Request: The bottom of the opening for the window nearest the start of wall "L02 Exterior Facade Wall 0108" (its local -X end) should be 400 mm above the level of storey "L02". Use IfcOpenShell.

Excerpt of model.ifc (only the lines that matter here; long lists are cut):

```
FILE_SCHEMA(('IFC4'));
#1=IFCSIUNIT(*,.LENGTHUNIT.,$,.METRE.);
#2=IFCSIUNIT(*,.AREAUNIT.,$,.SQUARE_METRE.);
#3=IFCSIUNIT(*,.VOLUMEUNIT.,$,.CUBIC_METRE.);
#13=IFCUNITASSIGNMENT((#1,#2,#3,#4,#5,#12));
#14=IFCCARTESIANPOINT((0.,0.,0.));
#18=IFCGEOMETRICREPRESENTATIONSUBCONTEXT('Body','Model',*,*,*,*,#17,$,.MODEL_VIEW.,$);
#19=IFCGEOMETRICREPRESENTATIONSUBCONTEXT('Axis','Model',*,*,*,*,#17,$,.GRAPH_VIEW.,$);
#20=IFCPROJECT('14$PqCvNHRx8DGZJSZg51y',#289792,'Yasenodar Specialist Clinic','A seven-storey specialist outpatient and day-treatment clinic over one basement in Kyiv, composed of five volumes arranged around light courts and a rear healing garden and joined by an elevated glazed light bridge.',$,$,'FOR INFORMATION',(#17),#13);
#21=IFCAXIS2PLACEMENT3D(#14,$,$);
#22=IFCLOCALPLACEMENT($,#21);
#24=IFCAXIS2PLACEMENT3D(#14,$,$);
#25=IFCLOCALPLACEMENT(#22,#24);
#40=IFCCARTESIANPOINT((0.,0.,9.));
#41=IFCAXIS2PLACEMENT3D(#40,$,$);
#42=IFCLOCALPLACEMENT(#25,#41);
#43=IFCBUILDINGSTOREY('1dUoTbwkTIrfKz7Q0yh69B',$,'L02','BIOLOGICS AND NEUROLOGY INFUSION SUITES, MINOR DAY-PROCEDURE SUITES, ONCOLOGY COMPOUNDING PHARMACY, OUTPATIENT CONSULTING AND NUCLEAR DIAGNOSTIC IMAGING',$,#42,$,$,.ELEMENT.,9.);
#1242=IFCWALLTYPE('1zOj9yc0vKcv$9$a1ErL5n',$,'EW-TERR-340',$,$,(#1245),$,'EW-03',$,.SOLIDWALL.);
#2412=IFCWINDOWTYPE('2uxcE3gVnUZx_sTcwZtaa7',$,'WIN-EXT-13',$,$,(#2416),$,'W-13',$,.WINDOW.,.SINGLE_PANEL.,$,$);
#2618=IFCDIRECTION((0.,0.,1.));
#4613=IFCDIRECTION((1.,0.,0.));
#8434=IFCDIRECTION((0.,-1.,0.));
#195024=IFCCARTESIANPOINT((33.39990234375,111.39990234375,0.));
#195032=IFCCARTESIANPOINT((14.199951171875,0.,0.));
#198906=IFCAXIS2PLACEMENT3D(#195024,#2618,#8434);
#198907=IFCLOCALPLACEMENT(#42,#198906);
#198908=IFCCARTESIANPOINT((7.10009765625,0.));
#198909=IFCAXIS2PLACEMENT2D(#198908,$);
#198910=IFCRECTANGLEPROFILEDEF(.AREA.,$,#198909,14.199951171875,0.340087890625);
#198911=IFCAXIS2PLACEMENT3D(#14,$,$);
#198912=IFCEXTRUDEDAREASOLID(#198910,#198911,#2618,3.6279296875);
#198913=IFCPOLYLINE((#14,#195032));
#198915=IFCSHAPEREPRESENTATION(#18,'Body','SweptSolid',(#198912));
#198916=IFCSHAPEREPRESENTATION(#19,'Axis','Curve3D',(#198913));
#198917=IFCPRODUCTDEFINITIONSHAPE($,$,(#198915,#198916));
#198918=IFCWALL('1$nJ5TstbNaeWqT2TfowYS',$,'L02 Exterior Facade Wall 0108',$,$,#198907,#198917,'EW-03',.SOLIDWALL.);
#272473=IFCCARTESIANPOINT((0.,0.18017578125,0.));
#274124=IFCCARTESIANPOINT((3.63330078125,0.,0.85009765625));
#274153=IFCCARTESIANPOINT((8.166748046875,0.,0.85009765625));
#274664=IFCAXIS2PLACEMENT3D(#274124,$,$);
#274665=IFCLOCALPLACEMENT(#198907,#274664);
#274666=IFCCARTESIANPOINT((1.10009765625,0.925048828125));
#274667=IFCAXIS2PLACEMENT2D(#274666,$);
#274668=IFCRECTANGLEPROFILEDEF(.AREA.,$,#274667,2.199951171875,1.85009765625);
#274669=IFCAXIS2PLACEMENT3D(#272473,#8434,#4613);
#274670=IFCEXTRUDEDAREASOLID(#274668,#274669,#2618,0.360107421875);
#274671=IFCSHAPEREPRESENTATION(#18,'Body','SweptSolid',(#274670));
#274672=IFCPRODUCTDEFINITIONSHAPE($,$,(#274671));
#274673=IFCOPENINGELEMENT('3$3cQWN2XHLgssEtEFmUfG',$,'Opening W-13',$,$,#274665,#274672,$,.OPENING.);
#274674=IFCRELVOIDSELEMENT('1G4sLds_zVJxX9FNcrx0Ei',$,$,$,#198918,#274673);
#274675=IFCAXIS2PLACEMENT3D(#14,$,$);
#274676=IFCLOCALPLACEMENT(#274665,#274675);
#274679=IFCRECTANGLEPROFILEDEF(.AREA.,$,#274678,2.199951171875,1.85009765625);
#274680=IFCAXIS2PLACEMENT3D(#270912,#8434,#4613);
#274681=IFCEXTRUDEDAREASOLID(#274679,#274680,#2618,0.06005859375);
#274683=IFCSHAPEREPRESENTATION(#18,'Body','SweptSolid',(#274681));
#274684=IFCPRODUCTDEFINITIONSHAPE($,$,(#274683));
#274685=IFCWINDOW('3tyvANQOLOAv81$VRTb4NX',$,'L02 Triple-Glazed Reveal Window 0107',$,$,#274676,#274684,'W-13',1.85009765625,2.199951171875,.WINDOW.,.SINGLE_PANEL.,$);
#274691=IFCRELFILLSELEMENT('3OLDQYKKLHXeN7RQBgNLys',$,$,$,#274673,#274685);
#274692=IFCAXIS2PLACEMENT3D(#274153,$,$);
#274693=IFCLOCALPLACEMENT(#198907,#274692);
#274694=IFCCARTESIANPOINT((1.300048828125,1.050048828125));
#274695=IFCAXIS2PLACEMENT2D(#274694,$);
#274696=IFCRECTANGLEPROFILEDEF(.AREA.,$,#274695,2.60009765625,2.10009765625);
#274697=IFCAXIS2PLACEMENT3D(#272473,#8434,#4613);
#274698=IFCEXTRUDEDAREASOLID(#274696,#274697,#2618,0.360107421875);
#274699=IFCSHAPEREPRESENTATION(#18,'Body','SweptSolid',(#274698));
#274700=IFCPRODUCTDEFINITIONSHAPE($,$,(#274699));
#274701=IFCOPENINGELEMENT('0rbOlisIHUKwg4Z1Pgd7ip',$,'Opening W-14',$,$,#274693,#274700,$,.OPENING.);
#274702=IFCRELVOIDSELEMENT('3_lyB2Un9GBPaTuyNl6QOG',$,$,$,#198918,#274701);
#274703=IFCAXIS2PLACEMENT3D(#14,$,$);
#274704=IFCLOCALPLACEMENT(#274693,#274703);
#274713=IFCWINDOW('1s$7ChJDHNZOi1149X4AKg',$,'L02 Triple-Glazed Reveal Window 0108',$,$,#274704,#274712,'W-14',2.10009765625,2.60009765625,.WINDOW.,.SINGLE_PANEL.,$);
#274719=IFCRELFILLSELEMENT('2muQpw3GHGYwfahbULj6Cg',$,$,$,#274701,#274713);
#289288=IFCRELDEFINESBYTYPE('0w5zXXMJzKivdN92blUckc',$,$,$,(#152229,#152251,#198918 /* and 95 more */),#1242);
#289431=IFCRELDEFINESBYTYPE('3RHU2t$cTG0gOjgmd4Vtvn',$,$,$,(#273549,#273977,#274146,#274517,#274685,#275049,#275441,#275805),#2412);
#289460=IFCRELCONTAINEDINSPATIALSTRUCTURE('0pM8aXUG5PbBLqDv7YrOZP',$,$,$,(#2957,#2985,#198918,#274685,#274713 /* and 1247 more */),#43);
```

```python
import numpy as np
import ifcopenshell
import ifcopenshell.api.geometry
import ifcopenshell.geom
import ifcopenshell.util.element
import ifcopenshell.util.placement
import ifcopenshell.util.shape
import ifcopenshell.util.unit

model = ifcopenshell.open("model.ifc")
unit_scale = ifcopenshell.util.unit.calculate_unit_scale(model)

window = model.by_guid("3tyvANQOLOAv81$VRTb4NX")
opening = window.FillsVoids[0].RelatingOpeningElement
storey = ifcopenshell.util.element.get_container(window, ifc_class="IfcBuildingStorey")
level = ifcopenshell.util.placement.get_local_placement(storey.ObjectPlacement)[2, 3]

# The opening's origin need not be at the sill, so measure its lowest point.
shape = ifcopenshell.geom.create_shape(ifcopenshell.geom.settings(), opening)
bottom = ifcopenshell.util.shape.get_shape_bottom_elevation(shape, shape.geometry) / unit_scale
dz = level + 0.4 - bottom

shift = np.array([0.0, 0.0, dz])
# The window is placed relative to its opening, so it follows when the opening moves.
matrix = ifcopenshell.util.placement.get_local_placement(opening.ObjectPlacement)
matrix[:3, 3] += shift
ifcopenshell.api.geometry.edit_object_placement(
    model, product=opening, matrix=matrix, is_si=False, should_transform_children=True
)

print(f"moved by {dz * unit_scale:+.3f} m")

model.write("model_v2.ifc")
```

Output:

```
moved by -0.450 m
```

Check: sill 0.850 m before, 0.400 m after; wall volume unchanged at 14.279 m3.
